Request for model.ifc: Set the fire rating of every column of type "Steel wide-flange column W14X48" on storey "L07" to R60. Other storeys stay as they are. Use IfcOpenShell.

First a look at what the model holds.

```python
import ifcopenshell
import ifcopenshell.util.element

model = ifcopenshell.open("model.ifc")
print(model.schema)
storey = next(s for s in model.by_type("IfcBuildingStorey") if s.Name == "L07")
columns = [e for e in ifcopenshell.util.element.get_decomposition(storey) if e.is_a("IfcColumn")]
seen = {}
for e in columns:
    element_type = ifcopenshell.util.element.get_type(e)
    key = (element_type.Name if element_type != e and element_type else None, ifcopenshell.util.element.get_pset(e, "Pset_ColumnCommon", "FireRating"))
    seen[key] = seen.get(key, 0) + 1
for (name, value), count in sorted(seen.items(), key=str):
    print(count, "x", name, "|", value)
```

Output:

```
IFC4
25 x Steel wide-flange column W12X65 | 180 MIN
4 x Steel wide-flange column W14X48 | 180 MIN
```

```python
import ifcopenshell
import ifcopenshell.api.pset
import ifcopenshell.util.element

model = ifcopenshell.open("model.ifc")

storey = next(s for s in model.by_type("IfcBuildingStorey") if s.Name == "L07")
columns = [e for e in ifcopenshell.util.element.get_decomposition(storey) if e.is_a("IfcColumn")]

count = 0
for e in columns:
    element_type = ifcopenshell.util.element.get_type(e)
    if element_type in (None, e) or element_type.Name != "Steel wide-flange column W14X48":
        continue
    # add_pset returns the element's existing set when there is one.
    pset = ifcopenshell.api.pset.add_pset(model, product=e, name="Pset_ColumnCommon")
    ifcopenshell.api.pset.edit_pset(model, pset=pset, properties={"FireRating": "R60"})
    count += 1

print(count, "columns updated")

model.write("model_v2.ifc")
```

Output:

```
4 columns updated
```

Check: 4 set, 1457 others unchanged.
